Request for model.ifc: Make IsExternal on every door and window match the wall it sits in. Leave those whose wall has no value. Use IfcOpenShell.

First a look at what the model holds.

```python
import ifcopenshell
import ifcopenshell.util.element

model = ifcopenshell.open("model.ifc")
print(model.schema)
seen = {}
for e in model.by_type("IfcDoor") + model.by_type("IfcWindow"):
    if not e.FillsVoids:
        continue
    host = e.FillsVoids[0].RelatingOpeningElement.VoidsElements[0].RelatingBuildingElement
    own = ifcopenshell.util.element.get_pset(e, f"Pset_{e.is_a()[3:].removesuffix('StandardCase')}Common", "IsExternal")
    wall = ifcopenshell.util.element.get_pset(host, "Pset_WallCommon", "IsExternal")
    seen[e.is_a(), own, wall] = seen.get((e.is_a(), own, wall), 0) + 1
for (cls, own, wall), count in sorted(seen.items(), key=str):
    print(count, cls, "IsExternal:", own, "| host wall:", wall)
```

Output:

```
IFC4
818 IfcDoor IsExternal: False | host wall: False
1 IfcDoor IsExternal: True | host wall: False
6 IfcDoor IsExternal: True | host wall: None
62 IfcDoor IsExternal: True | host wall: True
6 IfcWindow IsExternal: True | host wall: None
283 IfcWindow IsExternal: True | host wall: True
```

```python
import ifcopenshell
import ifcopenshell.api.pset
import ifcopenshell.util.element

model = ifcopenshell.open("model.ifc")

count = 0
for ifc_class, pset_name in (("IfcDoor", "Pset_DoorCommon"), ("IfcWindow", "Pset_WindowCommon")):
    for e in model.by_type(ifc_class):
        if not e.FillsVoids:
            continue
        host = e.FillsVoids[0].RelatingOpeningElement.VoidsElements[0].RelatingBuildingElement
        external = ifcopenshell.util.element.get_pset(host, "Pset_WallCommon", "IsExternal")
        if external is None or ifcopenshell.util.element.get_pset(e, pset_name, "IsExternal") == external:
            continue
        pset = ifcopenshell.api.pset.add_pset(model, product=e, name=pset_name)
        ifcopenshell.api.pset.edit_pset(model, pset=pset, properties={"IsExternal": external})
        count += 1

print(count, "updated")

model.write("model_v2.ifc")
```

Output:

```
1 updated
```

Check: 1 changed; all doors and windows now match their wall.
